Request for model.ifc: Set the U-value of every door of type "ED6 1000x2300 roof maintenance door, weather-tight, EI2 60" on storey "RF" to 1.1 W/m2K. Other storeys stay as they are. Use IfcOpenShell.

First a look at what the model holds.

```python
import ifcopenshell
import ifcopenshell.util.element

model = ifcopenshell.open("model.ifc")
print(model.schema)
storey = next(s for s in model.by_type("IfcBuildingStorey") if s.Name == "RF")
doors = [e for e in ifcopenshell.util.element.get_decomposition(storey) if e.is_a("IfcDoor")]
seen = {}
for e in doors:
    element_type = ifcopenshell.util.element.get_type(e)
    key = (element_type.Name if element_type != e and element_type else None, ifcopenshell.util.element.get_pset(e, "Pset_DoorCommon", "ThermalTransmittance"))
    seen[key] = seen.get(key, 0) + 1
for (name, value), count in sorted(seen.items(), key=str):
    print(count, "x", name, "|", value)
```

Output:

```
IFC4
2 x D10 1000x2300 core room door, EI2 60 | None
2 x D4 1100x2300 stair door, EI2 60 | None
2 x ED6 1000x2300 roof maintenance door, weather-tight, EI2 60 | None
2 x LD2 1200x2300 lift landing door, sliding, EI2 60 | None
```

```python
import ifcopenshell
import ifcopenshell.api.pset
import ifcopenshell.util.element

model = ifcopenshell.open("model.ifc")

storey = next(s for s in model.by_type("IfcBuildingStorey") if s.Name == "RF")
doors = [e for e in ifcopenshell.util.element.get_decomposition(storey) if e.is_a("IfcDoor")]

count = 0
for e in doors:
    element_type = ifcopenshell.util.element.get_type(e)
    if element_type in (None, e) or element_type.Name != "ED6 1000x2300 roof maintenance door, weather-tight, EI2 60":
        continue
    # add_pset returns the element's existing set when there is one.
    pset = ifcopenshell.api.pset.add_pset(model, product=e, name="Pset_DoorCommon")
    ifcopenshell.api.pset.edit_pset(model, pset=pset, properties={"ThermalTransmittance": 1.1})
    count += 1

print(count, "doors updated")

model.write("model_rev.ifc")
```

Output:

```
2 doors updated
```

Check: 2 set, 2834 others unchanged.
